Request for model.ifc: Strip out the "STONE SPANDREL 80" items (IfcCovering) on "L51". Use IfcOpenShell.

First a look at what the model holds.

```python
import ifcopenshell
import ifcopenshell.util.element

model = ifcopenshell.open("model.ifc")
print(model.schema)
storey = next(s for s in model.by_type("IfcBuildingStorey") if s.Name == "L51")
coverings = [e for e in ifcopenshell.util.element.get_decomposition(storey) if e.is_a("IfcCovering")]
seen = {}
for e in coverings:
    element_type = ifcopenshell.util.element.get_type(e)
    name = element_type.Name if element_type not in (None, e) else None
    seen[name] = seen.get(name, 0) + 1
for name, count in sorted(seen.items(), key=str):
    print(count, "x", name)
```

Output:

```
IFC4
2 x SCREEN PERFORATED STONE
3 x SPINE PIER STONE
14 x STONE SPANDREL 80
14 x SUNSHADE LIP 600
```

```python
import ifcopenshell
import ifcopenshell.api.root
import ifcopenshell.util.element

model = ifcopenshell.open("model.ifc")

storey = next(s for s in model.by_type("IfcBuildingStorey") if s.Name == "L51")
coverings = [e for e in ifcopenshell.util.element.get_decomposition(storey) if e.is_a("IfcCovering")]
targets = [e for e in coverings if (t := ifcopenshell.util.element.get_type(e)) not in (None, e) and t.Name == "STONE SPANDREL 80"]

for e in targets:
    ifcopenshell.api.root.remove_product(model, product=e)
print(len(targets), "removed")

model.write("model_v2.ifc")
```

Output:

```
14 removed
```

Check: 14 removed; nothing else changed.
